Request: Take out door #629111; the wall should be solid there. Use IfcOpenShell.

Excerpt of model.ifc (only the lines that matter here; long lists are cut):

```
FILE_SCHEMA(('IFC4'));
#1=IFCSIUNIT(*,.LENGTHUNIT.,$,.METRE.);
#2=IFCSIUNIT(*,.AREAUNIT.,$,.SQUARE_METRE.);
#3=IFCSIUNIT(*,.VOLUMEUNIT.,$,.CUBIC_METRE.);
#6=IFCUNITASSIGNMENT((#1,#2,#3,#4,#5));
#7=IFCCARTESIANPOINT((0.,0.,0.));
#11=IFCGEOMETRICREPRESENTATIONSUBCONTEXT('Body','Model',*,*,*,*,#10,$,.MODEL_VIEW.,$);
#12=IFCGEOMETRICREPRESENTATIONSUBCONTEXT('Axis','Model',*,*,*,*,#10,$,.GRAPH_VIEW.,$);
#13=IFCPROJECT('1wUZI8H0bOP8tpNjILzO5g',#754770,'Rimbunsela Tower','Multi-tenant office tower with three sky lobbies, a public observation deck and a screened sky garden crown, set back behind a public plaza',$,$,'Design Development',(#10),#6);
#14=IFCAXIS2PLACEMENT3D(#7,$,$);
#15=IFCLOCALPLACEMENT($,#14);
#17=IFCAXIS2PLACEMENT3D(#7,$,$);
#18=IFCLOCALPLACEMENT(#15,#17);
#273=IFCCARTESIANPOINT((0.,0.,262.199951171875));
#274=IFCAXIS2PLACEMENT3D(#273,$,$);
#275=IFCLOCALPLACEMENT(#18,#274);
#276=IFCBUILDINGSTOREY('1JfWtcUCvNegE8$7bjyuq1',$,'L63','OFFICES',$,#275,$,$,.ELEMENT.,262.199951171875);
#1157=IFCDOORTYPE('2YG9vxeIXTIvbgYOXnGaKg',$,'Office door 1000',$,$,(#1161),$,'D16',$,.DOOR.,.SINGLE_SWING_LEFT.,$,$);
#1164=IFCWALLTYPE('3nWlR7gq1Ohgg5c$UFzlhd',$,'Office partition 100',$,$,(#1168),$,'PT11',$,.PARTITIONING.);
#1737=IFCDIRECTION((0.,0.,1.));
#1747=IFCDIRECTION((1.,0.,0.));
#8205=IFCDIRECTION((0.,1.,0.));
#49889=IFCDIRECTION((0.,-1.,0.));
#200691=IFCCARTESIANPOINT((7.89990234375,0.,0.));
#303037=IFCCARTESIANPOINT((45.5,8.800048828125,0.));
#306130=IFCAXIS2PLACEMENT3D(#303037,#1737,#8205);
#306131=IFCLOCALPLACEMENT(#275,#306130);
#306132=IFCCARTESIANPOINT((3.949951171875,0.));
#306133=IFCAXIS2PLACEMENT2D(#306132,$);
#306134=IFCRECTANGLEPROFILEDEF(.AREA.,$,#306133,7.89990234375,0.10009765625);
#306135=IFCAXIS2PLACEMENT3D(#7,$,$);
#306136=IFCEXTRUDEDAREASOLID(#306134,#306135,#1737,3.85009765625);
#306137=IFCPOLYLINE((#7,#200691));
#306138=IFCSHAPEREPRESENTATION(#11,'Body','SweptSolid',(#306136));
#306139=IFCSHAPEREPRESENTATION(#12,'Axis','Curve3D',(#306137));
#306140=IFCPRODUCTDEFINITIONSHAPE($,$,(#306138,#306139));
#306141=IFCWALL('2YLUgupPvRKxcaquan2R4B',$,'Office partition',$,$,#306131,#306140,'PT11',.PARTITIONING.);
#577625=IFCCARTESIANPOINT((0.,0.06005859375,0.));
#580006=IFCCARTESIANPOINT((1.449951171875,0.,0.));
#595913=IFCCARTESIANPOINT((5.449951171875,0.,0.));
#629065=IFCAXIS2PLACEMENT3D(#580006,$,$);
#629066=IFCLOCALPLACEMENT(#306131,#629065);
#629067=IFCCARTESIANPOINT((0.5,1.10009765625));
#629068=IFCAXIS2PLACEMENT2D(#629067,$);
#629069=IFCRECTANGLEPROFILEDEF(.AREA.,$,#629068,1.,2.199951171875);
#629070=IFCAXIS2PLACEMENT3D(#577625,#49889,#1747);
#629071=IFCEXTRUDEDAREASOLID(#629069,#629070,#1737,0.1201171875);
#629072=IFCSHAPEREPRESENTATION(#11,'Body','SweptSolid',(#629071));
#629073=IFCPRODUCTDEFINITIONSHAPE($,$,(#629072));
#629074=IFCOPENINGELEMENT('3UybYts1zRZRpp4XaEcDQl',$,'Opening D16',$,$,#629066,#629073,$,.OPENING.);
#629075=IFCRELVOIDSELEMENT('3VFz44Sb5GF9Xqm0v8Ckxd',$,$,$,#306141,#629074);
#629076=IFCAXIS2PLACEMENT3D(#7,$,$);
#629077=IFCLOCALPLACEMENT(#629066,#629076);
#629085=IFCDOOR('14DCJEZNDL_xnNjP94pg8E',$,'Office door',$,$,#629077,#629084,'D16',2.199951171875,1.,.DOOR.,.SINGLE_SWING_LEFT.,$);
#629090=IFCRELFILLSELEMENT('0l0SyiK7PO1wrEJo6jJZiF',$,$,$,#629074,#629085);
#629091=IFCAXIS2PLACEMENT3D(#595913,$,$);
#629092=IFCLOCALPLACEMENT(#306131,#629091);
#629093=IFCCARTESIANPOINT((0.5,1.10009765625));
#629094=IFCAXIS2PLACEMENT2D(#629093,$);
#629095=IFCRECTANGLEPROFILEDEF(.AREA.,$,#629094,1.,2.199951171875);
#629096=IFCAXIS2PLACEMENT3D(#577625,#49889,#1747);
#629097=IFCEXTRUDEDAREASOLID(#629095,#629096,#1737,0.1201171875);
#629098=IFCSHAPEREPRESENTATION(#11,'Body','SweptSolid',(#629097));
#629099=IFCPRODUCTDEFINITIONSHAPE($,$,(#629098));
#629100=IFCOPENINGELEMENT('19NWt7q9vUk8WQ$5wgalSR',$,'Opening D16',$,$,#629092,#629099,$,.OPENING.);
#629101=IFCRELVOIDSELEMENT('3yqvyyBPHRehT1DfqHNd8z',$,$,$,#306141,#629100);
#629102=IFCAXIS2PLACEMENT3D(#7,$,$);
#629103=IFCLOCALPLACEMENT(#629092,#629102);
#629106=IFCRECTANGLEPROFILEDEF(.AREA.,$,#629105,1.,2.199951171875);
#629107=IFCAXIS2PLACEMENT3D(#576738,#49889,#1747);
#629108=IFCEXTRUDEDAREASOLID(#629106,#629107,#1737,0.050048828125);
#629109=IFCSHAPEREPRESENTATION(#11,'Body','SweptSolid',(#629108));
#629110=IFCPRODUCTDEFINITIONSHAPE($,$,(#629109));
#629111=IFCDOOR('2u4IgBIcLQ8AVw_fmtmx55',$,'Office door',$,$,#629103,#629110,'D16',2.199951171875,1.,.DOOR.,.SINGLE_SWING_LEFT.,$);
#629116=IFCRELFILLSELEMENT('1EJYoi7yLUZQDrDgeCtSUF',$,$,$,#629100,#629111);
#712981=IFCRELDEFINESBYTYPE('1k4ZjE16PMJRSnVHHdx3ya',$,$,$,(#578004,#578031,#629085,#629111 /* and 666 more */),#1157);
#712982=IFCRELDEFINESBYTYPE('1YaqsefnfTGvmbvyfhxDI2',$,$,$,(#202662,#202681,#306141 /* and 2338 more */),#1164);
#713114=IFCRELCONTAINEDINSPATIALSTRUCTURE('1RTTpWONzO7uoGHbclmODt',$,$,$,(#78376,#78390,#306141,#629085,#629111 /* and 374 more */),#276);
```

```python
import ifcopenshell
import ifcopenshell.api.feature
import ifcopenshell.api.root
import ifcopenshell.geom
import ifcopenshell.util.shape

model = ifcopenshell.open("model.ifc")
settings = ifcopenshell.geom.settings()


def volume(element):
    """Net volume in cubic metres, openings subtracted."""
    shape = ifcopenshell.geom.create_shape(settings, element)
    return ifcopenshell.util.shape.get_volume(shape.geometry)


door = model.by_id(629111)
opening = door.FillsVoids[0].RelatingOpeningElement
wall = opening.VoidsElements[0].RelatingBuildingElement
before = volume(wall)

ifcopenshell.api.root.remove_product(model, product=door)
ifcopenshell.api.feature.remove_feature(model, feature=opening)

after = volume(wall)

print(f"wall volume {before:.3f} -> {after:.3f} m3")

model.write("model_v2.ifc")
```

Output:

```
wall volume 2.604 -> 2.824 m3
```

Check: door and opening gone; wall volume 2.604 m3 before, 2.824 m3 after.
